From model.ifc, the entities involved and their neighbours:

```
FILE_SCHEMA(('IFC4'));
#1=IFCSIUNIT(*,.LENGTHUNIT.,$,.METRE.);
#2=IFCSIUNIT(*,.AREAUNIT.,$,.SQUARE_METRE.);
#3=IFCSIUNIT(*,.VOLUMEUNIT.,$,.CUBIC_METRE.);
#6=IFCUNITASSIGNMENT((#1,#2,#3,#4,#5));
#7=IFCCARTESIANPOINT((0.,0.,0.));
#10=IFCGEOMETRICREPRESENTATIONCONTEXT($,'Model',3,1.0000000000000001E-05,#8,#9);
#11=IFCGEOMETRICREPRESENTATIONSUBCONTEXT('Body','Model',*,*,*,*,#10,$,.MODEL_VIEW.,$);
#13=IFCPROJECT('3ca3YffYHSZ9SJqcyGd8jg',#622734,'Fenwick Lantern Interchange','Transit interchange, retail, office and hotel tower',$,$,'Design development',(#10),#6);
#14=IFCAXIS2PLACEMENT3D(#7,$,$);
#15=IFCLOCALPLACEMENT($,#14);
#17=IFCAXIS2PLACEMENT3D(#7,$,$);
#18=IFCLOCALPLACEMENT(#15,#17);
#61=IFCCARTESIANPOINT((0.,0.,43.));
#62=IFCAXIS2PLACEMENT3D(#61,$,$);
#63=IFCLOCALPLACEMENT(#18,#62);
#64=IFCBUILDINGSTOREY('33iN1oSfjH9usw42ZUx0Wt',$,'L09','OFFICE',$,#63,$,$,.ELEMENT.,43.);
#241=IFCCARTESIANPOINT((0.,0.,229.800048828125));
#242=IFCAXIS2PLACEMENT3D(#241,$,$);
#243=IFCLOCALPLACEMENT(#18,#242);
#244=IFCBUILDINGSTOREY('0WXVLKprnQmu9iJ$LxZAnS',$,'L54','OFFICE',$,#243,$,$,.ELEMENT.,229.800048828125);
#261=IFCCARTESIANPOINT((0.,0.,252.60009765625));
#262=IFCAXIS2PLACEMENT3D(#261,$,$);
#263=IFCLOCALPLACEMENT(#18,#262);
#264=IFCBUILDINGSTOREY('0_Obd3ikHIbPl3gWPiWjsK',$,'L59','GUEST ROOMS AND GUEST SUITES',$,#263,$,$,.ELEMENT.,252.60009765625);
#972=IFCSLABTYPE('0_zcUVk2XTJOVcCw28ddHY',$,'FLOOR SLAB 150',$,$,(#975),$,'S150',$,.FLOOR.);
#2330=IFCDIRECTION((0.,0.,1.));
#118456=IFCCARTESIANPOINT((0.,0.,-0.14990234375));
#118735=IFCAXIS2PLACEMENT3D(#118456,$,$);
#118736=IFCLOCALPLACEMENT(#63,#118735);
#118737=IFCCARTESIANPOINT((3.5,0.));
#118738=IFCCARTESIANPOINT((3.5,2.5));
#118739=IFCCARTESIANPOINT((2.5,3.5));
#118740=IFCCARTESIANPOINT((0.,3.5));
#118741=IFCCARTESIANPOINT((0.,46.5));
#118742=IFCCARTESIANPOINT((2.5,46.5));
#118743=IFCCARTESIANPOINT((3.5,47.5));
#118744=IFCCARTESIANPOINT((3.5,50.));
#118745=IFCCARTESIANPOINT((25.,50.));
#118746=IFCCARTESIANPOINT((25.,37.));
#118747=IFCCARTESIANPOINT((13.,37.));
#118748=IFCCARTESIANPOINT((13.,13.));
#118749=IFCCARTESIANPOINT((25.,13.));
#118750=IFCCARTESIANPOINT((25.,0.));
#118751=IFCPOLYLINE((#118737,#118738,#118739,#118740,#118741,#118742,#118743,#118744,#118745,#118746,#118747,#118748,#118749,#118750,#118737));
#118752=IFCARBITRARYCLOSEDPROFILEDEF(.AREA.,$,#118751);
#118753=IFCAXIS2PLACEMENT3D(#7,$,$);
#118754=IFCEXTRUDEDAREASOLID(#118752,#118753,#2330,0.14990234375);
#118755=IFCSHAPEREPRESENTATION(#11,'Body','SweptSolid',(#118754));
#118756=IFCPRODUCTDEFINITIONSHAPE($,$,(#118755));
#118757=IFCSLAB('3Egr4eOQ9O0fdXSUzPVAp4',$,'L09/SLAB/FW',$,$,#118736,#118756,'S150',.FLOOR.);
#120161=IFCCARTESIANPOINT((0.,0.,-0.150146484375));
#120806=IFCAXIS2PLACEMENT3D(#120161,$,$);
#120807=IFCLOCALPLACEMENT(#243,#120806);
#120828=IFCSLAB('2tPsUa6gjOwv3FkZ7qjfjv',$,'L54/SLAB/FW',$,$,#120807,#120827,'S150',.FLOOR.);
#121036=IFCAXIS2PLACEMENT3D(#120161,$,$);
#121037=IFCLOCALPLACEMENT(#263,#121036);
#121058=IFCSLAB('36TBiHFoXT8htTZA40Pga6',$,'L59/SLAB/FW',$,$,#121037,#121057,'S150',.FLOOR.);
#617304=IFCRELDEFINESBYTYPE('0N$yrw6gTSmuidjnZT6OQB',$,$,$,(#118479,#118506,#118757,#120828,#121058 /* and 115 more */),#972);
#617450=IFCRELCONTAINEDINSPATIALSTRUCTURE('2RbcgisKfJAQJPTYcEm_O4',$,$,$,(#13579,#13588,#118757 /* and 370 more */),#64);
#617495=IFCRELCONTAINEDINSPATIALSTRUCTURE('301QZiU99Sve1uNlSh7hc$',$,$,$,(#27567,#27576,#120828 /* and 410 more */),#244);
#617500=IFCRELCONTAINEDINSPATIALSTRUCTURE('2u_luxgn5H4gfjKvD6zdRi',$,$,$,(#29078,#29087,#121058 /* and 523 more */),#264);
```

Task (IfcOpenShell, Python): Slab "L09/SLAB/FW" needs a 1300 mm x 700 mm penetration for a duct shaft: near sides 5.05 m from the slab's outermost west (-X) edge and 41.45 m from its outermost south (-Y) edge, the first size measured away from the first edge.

```python
import numpy as np
import ifcopenshell
import ifcopenshell.api.feature
import ifcopenshell.api.geometry
import ifcopenshell.api.root
import ifcopenshell.geom
import ifcopenshell.util.placement
import ifcopenshell.util.representation
import ifcopenshell.util.shape
import ifcopenshell.util.unit

model = ifcopenshell.open("model.ifc")
unit_scale = ifcopenshell.util.unit.calculate_unit_scale(model)
settings = ifcopenshell.geom.settings()


def volume(element):
    """Net volume in cubic metres, openings subtracted."""
    shape = ifcopenshell.geom.create_shape(settings, element)
    return ifcopenshell.util.shape.get_volume(shape.geometry)


slab = model.by_id(118757)
before = volume(slab)

# Extent in the slab's own axes, in metres. The edges named are its -X and -Y sides.
slab_shape = ifcopenshell.geom.create_shape(settings, slab)
vertices = ifcopenshell.util.shape.get_vertices(slab_shape.geometry)
x_min, y_min, bottom = vertices.min(axis=0)
top = vertices[:, 2].max()

opening = ifcopenshell.api.root.create_entity(model, ifc_class="IfcOpeningElement", name="Duct shaft opening", predefined_type="OPENING")
context = ifcopenshell.util.representation.get_context(model, "Model", "Body", "MODEL_VIEW")
width, depth = 1.3, 0.7
outline = [(0.0, 0.0), (width, 0.0), (width, depth), (0.0, depth), (0.0, 0.0)]
# Overshoot both faces by 50 mm so the cut is clean.
shape = ifcopenshell.api.geometry.add_slab_representation(
    model, context=context, depth=top - bottom + 0.1, polyline=outline
)
ifcopenshell.api.geometry.assign_representation(model, product=opening, representation=shape)

matrix = ifcopenshell.util.placement.get_local_placement(slab.ObjectPlacement)
matrix[:, 3] = matrix @ np.append(np.array([x_min + 5.05, y_min + 41.45, bottom - 0.05]) / unit_scale, 1.0)
ifcopenshell.api.geometry.edit_object_placement(model, product=opening, matrix=matrix, is_si=False)
ifcopenshell.api.feature.add_feature(model, feature=opening, element=slab)

after = volume(slab)

print(f"slab volume {before:.3f} -> {after:.3f} m3")

model.write("model_edited.ifc")
```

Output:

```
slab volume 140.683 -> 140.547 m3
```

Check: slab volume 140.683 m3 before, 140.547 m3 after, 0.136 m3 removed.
